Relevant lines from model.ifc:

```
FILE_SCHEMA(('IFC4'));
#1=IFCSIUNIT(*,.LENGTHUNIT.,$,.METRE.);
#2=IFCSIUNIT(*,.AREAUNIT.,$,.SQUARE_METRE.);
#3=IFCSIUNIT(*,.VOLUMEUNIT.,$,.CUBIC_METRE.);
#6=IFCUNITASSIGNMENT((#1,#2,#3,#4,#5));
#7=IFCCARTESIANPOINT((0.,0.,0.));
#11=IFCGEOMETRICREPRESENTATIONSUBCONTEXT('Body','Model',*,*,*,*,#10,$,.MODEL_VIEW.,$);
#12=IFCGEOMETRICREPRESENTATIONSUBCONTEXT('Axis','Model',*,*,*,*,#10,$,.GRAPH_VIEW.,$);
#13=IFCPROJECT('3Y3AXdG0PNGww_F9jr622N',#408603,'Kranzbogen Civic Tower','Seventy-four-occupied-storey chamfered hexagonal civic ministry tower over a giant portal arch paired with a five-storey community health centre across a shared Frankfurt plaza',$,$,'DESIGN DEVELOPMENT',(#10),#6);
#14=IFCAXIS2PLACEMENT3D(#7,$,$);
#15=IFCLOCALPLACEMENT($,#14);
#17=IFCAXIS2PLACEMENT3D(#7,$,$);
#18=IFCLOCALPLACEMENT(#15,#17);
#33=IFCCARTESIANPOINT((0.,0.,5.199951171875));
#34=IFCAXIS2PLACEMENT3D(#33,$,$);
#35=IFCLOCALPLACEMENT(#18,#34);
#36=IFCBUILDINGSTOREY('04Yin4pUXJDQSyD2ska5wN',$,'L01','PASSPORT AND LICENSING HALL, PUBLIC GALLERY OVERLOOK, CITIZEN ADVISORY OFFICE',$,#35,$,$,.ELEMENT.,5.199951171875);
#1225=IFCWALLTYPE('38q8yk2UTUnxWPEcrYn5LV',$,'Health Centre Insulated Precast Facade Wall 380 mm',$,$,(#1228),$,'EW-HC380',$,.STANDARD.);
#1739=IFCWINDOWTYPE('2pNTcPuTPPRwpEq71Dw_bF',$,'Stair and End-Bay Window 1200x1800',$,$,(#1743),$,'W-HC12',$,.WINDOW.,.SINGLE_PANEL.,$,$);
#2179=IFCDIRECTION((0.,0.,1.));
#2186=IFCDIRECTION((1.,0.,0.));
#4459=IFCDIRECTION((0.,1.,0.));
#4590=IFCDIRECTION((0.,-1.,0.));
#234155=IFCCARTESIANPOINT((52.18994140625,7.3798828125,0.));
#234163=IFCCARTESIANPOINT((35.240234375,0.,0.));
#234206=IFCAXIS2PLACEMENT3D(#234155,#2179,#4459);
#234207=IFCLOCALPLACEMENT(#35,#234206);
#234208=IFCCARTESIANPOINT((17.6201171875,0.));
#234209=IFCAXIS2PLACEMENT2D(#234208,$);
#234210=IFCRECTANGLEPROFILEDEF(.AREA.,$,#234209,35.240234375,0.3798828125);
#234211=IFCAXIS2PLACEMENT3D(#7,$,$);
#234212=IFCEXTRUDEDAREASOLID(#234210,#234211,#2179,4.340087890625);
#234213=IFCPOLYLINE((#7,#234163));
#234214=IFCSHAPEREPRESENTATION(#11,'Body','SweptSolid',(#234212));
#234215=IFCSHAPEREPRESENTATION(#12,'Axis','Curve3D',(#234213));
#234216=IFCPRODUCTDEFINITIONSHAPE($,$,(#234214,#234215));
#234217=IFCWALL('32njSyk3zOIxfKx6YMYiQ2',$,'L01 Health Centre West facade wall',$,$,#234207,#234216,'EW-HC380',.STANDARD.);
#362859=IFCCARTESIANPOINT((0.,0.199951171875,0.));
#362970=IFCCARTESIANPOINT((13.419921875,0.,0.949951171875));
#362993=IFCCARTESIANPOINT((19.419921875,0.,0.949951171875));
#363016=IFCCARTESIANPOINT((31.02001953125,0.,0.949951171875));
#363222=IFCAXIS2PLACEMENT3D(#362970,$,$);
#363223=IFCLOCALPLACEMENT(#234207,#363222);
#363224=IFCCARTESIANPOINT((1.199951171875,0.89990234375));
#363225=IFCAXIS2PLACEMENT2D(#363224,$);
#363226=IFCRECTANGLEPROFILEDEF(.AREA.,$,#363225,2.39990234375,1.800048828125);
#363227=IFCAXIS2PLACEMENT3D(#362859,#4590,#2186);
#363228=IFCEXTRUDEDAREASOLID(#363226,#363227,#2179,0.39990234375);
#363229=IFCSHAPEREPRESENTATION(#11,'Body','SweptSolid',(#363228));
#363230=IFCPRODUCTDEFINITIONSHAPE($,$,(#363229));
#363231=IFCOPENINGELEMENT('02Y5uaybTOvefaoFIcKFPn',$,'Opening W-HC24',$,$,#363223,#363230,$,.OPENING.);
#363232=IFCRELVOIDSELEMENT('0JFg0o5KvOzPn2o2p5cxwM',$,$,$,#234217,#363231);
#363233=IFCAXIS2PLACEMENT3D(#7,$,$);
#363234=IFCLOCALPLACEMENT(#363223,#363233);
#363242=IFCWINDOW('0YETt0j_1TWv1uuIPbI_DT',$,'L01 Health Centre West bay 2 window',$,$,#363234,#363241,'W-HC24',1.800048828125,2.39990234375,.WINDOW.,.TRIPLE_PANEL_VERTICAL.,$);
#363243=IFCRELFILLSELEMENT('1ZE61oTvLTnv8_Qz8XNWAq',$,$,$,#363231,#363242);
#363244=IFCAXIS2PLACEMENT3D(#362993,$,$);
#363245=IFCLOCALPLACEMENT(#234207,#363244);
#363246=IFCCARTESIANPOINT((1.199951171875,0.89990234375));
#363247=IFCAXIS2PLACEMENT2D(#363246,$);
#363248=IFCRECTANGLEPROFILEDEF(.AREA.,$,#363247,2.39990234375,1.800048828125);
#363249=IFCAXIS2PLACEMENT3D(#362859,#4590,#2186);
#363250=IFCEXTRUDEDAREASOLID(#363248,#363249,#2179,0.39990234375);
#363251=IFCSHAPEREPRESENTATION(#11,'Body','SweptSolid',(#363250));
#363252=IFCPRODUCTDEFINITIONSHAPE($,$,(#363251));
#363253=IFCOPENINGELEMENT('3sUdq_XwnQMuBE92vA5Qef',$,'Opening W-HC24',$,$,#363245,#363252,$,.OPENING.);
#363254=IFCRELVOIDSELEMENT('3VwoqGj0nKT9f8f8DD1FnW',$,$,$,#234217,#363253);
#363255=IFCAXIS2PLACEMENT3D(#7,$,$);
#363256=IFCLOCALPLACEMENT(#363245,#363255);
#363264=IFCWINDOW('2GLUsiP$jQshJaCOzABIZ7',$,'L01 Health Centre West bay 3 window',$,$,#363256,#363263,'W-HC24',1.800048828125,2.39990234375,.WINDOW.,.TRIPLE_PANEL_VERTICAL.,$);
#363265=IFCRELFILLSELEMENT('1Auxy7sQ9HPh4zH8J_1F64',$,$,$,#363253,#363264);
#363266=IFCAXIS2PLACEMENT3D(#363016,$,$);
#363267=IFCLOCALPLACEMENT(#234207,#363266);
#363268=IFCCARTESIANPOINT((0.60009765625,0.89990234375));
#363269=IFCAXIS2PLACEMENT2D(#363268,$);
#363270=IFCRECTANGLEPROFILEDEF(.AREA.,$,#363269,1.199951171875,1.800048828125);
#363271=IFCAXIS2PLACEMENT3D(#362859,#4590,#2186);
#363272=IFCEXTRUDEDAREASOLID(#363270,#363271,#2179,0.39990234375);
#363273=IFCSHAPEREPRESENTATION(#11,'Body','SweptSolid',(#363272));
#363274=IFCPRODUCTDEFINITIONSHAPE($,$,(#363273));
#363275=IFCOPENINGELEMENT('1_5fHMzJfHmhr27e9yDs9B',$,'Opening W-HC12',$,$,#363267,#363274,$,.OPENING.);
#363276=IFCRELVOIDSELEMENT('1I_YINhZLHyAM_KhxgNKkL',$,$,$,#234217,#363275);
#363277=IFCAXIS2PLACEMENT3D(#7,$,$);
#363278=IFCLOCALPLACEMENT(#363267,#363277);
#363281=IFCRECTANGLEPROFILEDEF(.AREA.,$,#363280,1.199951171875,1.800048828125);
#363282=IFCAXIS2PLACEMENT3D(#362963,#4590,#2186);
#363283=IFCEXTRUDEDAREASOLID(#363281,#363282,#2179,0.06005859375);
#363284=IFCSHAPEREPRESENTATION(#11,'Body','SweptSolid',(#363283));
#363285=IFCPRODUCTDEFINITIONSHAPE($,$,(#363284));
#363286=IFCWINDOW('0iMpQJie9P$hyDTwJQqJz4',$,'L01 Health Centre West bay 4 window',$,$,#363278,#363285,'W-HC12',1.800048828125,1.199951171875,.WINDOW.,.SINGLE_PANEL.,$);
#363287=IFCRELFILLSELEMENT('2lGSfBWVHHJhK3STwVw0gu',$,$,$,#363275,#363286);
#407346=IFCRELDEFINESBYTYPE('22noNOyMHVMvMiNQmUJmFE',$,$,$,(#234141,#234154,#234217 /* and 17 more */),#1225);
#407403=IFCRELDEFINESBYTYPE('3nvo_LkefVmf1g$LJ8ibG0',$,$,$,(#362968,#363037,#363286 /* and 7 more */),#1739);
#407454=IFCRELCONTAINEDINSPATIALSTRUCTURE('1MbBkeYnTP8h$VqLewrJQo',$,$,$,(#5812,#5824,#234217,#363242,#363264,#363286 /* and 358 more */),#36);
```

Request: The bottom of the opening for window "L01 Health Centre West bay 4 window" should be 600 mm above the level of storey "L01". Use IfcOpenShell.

```python
import numpy as np
import ifcopenshell
import ifcopenshell.api.geometry
import ifcopenshell.geom
import ifcopenshell.util.element
import ifcopenshell.util.placement
import ifcopenshell.util.shape
import ifcopenshell.util.unit

model = ifcopenshell.open("model.ifc")
unit_scale = ifcopenshell.util.unit.calculate_unit_scale(model)

window = model.by_guid("0iMpQJie9P$hyDTwJQqJz4")
opening = window.FillsVoids[0].RelatingOpeningElement
storey = ifcopenshell.util.element.get_container(window, ifc_class="IfcBuildingStorey")
level = ifcopenshell.util.placement.get_local_placement(storey.ObjectPlacement)[2, 3]

# The opening's origin need not be at the sill, so measure its lowest point.
shape = ifcopenshell.geom.create_shape(ifcopenshell.geom.settings(), opening)
bottom = ifcopenshell.util.shape.get_shape_bottom_elevation(shape, shape.geometry) / unit_scale
dz = level + 0.6 / unit_scale - bottom

shift = np.array([0.0, 0.0, dz])
# The window is placed relative to its opening, so it follows when the opening moves.
matrix = ifcopenshell.util.placement.get_local_placement(opening.ObjectPlacement)
matrix[:3, 3] += shift
ifcopenshell.api.geometry.edit_object_placement(
    model, product=opening, matrix=matrix, is_si=False, should_transform_children=True
)

print(f"moved by {dz * unit_scale:+.3f} m")

model.write("model-out.ifc")
```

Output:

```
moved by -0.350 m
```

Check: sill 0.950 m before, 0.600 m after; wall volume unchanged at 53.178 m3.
